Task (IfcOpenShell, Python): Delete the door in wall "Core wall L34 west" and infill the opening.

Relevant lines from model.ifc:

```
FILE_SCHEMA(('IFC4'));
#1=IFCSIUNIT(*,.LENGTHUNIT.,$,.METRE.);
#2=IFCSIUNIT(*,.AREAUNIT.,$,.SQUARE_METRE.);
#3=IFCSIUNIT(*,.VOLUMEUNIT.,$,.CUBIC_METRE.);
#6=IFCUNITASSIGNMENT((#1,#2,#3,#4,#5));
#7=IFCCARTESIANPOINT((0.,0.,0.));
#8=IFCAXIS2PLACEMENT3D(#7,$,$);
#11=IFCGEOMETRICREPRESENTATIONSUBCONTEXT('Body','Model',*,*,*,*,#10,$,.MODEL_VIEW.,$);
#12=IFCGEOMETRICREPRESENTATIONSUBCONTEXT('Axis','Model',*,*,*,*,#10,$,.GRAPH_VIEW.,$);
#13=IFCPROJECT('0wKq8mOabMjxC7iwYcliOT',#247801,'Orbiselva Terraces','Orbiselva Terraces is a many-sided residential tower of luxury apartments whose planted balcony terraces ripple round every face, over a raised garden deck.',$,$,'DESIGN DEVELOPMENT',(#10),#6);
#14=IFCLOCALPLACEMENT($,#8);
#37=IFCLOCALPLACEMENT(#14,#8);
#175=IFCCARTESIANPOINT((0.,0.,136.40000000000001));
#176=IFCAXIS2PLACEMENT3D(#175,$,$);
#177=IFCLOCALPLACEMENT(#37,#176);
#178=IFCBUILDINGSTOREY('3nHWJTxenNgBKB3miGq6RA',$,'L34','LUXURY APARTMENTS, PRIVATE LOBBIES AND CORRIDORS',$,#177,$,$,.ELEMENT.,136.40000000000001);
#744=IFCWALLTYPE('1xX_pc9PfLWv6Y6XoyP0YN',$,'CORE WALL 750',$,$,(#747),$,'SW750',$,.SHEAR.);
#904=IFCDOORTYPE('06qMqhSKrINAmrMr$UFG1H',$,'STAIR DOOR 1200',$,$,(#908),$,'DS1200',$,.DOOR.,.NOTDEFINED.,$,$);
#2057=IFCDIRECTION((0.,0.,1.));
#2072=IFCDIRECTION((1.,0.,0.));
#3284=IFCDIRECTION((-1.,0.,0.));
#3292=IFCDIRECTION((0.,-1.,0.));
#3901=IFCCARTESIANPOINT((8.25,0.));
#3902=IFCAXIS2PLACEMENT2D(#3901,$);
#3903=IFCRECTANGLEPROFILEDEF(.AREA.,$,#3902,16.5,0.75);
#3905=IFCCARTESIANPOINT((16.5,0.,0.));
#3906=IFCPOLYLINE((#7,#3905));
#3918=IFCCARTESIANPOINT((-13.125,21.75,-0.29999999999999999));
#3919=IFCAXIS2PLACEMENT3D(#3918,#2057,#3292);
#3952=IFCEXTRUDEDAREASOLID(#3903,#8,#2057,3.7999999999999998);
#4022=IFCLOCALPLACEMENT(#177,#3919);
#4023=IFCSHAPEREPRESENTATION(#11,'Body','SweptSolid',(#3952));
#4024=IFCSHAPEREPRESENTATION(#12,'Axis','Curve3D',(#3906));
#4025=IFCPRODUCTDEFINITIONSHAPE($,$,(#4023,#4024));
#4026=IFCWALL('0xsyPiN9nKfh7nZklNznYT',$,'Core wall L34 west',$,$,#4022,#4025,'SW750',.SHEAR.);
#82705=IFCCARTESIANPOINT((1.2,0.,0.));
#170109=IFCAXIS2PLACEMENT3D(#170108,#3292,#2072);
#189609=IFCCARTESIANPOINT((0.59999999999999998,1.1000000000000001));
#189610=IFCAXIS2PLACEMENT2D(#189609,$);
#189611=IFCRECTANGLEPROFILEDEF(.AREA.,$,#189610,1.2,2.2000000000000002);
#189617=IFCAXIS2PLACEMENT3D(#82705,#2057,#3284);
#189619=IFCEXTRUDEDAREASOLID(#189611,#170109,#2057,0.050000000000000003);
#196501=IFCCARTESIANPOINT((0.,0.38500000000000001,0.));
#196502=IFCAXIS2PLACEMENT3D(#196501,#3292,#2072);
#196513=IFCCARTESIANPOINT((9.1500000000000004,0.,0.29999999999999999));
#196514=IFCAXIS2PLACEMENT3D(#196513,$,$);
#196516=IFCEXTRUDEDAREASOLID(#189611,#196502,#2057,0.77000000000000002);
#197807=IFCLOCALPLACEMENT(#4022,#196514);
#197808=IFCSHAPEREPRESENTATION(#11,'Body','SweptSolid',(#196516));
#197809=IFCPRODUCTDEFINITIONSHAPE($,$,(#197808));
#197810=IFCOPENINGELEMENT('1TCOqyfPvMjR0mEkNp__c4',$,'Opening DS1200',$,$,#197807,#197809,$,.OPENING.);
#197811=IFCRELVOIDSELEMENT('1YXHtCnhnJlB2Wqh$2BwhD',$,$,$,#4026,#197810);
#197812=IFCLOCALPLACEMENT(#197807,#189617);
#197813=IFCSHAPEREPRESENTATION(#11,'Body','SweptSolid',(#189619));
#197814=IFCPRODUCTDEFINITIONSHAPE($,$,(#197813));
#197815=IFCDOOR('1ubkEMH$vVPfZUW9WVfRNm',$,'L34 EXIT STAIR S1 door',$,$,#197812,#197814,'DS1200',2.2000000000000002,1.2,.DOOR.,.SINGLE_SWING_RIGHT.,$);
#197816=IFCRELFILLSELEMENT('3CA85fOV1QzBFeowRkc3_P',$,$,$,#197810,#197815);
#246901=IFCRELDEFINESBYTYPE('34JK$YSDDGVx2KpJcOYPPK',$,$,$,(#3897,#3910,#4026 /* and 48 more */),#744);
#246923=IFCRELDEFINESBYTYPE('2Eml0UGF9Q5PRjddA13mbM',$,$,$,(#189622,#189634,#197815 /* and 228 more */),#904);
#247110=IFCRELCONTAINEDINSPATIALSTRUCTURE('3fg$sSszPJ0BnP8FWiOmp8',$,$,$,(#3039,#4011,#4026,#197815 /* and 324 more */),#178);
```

```python
import ifcopenshell
import ifcopenshell.api.feature
import ifcopenshell.api.root
import ifcopenshell.geom
import ifcopenshell.util.shape

model = ifcopenshell.open("model.ifc")
settings = ifcopenshell.geom.settings()


def volume(element):
    """Net volume in cubic metres, openings subtracted."""
    shape = ifcopenshell.geom.create_shape(settings, element)
    return ifcopenshell.util.shape.get_volume(shape.geometry)


door = model.by_guid("1ubkEMH$vVPfZUW9WVfRNm")
opening = door.FillsVoids[0].RelatingOpeningElement
wall = opening.VoidsElements[0].RelatingBuildingElement
before = volume(wall)

ifcopenshell.api.root.remove_product(model, product=door)
ifcopenshell.api.feature.remove_feature(model, feature=opening)

after = volume(wall)

print(f"wall volume {before:.3f} -> {after:.3f} m3")

model.write("model-out.ifc")
```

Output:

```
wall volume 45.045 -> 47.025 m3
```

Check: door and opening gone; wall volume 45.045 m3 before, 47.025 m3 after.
